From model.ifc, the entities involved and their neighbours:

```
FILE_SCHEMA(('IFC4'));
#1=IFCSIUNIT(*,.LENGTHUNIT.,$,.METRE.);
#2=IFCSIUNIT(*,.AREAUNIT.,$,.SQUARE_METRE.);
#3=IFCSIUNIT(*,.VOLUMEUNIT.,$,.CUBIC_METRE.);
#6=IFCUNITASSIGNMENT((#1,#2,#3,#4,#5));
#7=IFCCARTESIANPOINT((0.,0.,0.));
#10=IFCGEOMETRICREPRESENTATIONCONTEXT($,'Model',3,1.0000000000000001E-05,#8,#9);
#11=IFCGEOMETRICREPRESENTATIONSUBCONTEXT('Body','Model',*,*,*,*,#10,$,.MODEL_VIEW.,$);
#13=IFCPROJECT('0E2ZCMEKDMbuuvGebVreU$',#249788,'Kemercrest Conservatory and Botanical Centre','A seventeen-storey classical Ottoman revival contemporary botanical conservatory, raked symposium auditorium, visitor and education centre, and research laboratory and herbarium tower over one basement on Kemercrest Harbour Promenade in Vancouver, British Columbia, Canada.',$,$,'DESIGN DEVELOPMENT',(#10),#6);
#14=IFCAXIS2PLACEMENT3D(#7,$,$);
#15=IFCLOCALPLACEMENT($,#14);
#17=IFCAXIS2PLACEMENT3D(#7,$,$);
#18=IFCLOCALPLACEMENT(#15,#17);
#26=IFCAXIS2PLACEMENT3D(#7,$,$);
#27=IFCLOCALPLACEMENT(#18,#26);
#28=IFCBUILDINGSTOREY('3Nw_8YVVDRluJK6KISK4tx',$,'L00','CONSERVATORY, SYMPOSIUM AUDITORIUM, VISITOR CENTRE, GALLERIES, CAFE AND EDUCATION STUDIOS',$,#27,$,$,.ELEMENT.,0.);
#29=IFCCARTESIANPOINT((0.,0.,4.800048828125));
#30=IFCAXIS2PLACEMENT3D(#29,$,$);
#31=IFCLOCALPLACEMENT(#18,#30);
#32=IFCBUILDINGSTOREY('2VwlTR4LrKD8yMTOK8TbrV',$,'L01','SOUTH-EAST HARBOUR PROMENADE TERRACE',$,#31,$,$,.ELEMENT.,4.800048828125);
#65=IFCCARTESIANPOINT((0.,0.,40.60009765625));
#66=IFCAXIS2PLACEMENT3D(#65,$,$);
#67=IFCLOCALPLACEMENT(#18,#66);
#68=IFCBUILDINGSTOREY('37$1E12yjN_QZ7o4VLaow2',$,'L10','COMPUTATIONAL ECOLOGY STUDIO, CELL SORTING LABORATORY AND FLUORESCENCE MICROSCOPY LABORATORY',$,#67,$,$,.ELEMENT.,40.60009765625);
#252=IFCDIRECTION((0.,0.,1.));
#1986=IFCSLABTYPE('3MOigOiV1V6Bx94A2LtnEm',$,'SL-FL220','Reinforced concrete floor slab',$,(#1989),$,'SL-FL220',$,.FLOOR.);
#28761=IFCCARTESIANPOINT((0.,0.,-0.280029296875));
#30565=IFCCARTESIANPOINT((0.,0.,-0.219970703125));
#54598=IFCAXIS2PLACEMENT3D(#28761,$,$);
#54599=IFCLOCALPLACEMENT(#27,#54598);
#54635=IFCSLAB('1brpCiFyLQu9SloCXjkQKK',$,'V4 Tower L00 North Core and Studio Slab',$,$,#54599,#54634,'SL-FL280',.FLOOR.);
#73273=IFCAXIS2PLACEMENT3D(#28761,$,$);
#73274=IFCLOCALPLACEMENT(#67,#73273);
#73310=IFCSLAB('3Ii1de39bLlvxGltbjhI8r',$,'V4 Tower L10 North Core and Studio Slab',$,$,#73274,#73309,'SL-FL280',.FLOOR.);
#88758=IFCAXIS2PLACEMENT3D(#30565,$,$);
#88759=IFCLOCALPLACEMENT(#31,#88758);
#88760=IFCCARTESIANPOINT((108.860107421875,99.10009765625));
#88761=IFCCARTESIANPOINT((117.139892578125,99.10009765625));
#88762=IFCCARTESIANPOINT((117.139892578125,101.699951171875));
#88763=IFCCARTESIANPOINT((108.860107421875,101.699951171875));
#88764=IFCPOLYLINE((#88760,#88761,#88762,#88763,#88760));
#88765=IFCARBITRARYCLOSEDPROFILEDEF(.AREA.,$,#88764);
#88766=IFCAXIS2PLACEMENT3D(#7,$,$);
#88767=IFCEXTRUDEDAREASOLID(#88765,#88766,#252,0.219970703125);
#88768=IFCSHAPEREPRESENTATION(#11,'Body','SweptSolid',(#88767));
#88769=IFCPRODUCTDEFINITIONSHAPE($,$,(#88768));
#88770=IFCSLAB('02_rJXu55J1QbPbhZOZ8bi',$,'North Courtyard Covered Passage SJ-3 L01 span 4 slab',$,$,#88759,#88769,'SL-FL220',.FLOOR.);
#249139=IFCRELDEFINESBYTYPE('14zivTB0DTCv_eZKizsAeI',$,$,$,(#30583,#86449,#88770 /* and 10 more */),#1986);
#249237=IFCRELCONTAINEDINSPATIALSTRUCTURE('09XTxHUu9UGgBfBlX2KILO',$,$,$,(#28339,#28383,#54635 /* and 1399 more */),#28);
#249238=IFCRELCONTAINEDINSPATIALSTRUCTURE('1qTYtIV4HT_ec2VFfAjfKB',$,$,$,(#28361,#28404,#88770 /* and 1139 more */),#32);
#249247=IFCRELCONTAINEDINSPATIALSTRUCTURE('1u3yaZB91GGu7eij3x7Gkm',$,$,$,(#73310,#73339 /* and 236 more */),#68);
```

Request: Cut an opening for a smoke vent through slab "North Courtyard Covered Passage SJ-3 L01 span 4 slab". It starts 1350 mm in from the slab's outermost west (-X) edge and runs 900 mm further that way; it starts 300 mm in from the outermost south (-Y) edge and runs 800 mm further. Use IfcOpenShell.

```python
import numpy as np
import ifcopenshell
import ifcopenshell.api.feature
import ifcopenshell.api.geometry
import ifcopenshell.api.root
import ifcopenshell.geom
import ifcopenshell.util.placement
import ifcopenshell.util.representation
import ifcopenshell.util.shape
import ifcopenshell.util.unit

model = ifcopenshell.open("model.ifc")
unit_scale = ifcopenshell.util.unit.calculate_unit_scale(model)
settings = ifcopenshell.geom.settings()


def volume(element):
    """Net volume in cubic metres, openings subtracted."""
    shape = ifcopenshell.geom.create_shape(settings, element)
    return ifcopenshell.util.shape.get_volume(shape.geometry)


slab = model.by_guid("02_rJXu55J1QbPbhZOZ8bi")
before = volume(slab)

# Extent in the slab's own axes, in metres. The edges named are its -X and -Y sides.
slab_shape = ifcopenshell.geom.create_shape(settings, slab)
vertices = ifcopenshell.util.shape.get_vertices(slab_shape.geometry)
x_min, y_min, bottom = vertices.min(axis=0)
top = vertices[:, 2].max()

opening = ifcopenshell.api.root.create_entity(model, ifc_class="IfcOpeningElement", name="Smoke vent opening", predefined_type="OPENING")
context = ifcopenshell.util.representation.get_context(model, "Model", "Body", "MODEL_VIEW")
width, depth = 0.9, 0.8
outline = [(0.0, 0.0), (width, 0.0), (width, depth), (0.0, depth), (0.0, 0.0)]
# Overshoot both faces by 50 mm so the cut is clean.
shape = ifcopenshell.api.geometry.add_slab_representation(
    model, context=context, depth=top - bottom + 0.1, polyline=outline
)
ifcopenshell.api.geometry.assign_representation(model, product=opening, representation=shape)

matrix = ifcopenshell.util.placement.get_local_placement(slab.ObjectPlacement)
matrix[:, 3] = matrix @ np.append(np.array([x_min + 1.35, y_min + 0.3, bottom - 0.05]) / unit_scale, 1.0)
ifcopenshell.api.geometry.edit_object_placement(model, product=opening, matrix=matrix, is_si=False)
ifcopenshell.api.feature.add_feature(model, feature=opening, element=slab)

after = volume(slab)

print(f"slab volume {before:.3f} -> {after:.3f} m3")

model.write("model-out.ifc")
```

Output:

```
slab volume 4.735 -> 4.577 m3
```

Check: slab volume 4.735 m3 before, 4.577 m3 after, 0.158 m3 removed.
